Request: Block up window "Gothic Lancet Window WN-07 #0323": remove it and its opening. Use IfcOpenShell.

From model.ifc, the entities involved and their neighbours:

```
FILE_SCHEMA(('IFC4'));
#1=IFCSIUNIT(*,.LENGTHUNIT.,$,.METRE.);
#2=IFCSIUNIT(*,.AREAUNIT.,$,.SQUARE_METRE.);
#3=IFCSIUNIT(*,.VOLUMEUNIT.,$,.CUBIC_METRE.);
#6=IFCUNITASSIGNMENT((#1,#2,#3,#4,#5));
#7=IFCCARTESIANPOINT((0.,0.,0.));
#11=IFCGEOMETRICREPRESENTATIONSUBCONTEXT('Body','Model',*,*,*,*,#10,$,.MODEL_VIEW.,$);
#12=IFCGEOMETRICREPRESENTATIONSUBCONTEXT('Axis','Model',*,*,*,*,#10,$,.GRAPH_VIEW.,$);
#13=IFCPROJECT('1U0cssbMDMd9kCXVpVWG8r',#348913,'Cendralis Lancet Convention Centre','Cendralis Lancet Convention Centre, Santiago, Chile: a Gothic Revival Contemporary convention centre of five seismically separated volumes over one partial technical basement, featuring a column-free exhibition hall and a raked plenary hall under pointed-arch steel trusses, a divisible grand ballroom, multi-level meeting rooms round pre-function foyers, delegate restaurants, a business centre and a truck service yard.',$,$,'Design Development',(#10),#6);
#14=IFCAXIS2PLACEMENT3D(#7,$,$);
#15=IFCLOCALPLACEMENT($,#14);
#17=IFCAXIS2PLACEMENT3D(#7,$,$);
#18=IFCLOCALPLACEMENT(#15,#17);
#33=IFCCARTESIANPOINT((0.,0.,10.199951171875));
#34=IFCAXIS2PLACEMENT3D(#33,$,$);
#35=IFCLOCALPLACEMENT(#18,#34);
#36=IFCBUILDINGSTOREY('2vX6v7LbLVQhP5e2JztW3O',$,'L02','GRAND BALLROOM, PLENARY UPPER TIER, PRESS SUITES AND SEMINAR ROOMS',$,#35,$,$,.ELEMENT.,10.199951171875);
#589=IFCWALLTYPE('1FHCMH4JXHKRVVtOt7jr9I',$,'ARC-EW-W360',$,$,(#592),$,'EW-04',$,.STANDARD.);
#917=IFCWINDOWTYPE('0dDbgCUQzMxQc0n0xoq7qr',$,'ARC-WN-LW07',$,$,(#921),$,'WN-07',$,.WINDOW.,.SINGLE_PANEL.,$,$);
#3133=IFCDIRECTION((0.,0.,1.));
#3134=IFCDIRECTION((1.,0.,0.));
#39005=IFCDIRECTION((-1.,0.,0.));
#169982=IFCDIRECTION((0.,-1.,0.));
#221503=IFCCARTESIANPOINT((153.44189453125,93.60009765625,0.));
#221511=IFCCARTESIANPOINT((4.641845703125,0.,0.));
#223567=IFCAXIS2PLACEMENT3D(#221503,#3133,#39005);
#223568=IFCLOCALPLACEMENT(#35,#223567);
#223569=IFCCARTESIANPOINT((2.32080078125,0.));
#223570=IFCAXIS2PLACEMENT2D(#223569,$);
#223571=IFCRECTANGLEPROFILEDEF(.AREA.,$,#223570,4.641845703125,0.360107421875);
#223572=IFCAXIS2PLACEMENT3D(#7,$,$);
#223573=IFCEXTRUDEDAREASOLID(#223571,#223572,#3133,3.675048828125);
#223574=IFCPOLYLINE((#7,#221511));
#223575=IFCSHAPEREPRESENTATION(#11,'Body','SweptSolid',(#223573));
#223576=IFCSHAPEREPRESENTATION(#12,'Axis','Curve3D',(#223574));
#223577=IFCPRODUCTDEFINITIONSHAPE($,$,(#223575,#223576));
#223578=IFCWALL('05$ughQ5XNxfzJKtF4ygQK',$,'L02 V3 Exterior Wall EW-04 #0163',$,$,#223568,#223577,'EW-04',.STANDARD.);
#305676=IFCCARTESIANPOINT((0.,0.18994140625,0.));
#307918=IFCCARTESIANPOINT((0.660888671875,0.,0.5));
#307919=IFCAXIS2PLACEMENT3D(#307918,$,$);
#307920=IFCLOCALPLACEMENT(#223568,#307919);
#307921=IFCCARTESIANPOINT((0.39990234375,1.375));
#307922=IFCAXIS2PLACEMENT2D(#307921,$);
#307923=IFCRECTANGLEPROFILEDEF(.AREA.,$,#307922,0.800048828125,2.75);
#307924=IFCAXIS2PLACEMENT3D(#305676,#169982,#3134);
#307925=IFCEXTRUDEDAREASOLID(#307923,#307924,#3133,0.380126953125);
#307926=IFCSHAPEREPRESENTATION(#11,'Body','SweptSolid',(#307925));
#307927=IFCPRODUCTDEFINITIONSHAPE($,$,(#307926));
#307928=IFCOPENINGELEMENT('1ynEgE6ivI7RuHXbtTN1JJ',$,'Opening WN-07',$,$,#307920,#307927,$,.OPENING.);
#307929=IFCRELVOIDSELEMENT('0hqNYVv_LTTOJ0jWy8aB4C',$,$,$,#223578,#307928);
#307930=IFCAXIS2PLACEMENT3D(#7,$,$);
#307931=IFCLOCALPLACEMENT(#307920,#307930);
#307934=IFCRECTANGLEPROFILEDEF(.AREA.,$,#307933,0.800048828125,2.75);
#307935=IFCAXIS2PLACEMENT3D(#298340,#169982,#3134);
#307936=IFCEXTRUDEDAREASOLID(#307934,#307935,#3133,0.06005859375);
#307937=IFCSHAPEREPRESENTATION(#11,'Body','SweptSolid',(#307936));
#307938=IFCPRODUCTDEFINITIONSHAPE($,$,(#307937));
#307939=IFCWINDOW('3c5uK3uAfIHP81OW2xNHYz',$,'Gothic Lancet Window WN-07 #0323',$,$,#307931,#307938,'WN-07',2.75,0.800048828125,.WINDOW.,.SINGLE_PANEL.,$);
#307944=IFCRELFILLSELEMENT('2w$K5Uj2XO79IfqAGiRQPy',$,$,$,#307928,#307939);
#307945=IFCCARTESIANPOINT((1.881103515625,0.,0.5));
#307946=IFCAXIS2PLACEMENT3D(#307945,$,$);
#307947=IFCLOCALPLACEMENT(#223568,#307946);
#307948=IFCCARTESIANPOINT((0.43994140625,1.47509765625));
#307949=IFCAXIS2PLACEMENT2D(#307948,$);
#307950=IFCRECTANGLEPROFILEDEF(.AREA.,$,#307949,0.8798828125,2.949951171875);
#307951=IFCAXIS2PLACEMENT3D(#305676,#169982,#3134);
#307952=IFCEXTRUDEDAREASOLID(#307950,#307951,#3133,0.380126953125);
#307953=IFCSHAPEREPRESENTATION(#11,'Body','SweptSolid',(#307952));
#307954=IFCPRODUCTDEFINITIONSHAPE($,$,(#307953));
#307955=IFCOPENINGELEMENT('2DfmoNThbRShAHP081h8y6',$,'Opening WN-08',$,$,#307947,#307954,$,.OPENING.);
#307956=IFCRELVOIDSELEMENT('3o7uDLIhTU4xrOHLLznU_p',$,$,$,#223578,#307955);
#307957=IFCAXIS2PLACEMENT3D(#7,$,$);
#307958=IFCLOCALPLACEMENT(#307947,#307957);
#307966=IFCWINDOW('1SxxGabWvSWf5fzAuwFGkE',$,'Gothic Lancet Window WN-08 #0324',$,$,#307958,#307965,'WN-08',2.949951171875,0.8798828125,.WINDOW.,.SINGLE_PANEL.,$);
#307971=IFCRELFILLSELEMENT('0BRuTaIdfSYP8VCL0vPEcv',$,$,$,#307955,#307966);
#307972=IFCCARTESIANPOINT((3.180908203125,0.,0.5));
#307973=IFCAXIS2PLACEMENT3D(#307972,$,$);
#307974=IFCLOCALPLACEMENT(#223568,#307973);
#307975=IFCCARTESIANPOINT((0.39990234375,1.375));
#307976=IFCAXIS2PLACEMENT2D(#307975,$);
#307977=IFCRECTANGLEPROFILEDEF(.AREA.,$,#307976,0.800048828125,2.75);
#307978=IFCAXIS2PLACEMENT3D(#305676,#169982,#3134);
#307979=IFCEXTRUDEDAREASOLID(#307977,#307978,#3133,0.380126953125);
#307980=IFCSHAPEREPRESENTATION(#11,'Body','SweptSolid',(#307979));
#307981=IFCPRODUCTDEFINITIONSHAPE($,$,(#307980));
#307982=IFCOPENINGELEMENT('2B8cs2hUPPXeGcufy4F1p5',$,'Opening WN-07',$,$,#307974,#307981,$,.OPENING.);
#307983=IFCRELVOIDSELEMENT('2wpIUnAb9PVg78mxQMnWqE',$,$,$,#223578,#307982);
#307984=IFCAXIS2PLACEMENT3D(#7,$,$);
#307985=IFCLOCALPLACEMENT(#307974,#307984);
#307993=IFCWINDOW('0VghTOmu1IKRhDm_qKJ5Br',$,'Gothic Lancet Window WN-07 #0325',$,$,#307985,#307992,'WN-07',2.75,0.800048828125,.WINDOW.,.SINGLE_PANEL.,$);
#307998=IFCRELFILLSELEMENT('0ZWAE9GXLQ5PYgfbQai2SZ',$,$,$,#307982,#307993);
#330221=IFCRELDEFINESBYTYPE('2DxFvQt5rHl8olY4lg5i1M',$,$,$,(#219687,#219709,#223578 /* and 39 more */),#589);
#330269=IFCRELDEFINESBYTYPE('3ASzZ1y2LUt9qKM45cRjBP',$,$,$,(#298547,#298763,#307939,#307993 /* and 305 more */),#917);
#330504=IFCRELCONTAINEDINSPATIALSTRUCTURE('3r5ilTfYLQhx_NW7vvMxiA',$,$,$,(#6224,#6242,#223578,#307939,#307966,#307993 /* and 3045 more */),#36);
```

```python
import ifcopenshell
import ifcopenshell.api.feature
import ifcopenshell.api.root
import ifcopenshell.geom
import ifcopenshell.util.shape

model = ifcopenshell.open("model.ifc")
settings = ifcopenshell.geom.settings()


def volume(element):
    """Net volume in cubic metres, openings subtracted."""
    shape = ifcopenshell.geom.create_shape(settings, element)
    return ifcopenshell.util.shape.get_volume(shape.geometry)


window = model.by_guid("3c5uK3uAfIHP81OW2xNHYz")
opening = window.FillsVoids[0].RelatingOpeningElement
wall = opening.VoidsElements[0].RelatingBuildingElement
before = volume(wall)

ifcopenshell.api.root.remove_product(model, product=window)
ifcopenshell.api.feature.remove_feature(model, feature=opening)

after = volume(wall)

print(f"wall volume {before:.3f} -> {after:.3f} m3")

model.write("model_rev.ifc")
```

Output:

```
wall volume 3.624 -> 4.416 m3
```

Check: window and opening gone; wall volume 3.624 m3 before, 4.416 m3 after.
